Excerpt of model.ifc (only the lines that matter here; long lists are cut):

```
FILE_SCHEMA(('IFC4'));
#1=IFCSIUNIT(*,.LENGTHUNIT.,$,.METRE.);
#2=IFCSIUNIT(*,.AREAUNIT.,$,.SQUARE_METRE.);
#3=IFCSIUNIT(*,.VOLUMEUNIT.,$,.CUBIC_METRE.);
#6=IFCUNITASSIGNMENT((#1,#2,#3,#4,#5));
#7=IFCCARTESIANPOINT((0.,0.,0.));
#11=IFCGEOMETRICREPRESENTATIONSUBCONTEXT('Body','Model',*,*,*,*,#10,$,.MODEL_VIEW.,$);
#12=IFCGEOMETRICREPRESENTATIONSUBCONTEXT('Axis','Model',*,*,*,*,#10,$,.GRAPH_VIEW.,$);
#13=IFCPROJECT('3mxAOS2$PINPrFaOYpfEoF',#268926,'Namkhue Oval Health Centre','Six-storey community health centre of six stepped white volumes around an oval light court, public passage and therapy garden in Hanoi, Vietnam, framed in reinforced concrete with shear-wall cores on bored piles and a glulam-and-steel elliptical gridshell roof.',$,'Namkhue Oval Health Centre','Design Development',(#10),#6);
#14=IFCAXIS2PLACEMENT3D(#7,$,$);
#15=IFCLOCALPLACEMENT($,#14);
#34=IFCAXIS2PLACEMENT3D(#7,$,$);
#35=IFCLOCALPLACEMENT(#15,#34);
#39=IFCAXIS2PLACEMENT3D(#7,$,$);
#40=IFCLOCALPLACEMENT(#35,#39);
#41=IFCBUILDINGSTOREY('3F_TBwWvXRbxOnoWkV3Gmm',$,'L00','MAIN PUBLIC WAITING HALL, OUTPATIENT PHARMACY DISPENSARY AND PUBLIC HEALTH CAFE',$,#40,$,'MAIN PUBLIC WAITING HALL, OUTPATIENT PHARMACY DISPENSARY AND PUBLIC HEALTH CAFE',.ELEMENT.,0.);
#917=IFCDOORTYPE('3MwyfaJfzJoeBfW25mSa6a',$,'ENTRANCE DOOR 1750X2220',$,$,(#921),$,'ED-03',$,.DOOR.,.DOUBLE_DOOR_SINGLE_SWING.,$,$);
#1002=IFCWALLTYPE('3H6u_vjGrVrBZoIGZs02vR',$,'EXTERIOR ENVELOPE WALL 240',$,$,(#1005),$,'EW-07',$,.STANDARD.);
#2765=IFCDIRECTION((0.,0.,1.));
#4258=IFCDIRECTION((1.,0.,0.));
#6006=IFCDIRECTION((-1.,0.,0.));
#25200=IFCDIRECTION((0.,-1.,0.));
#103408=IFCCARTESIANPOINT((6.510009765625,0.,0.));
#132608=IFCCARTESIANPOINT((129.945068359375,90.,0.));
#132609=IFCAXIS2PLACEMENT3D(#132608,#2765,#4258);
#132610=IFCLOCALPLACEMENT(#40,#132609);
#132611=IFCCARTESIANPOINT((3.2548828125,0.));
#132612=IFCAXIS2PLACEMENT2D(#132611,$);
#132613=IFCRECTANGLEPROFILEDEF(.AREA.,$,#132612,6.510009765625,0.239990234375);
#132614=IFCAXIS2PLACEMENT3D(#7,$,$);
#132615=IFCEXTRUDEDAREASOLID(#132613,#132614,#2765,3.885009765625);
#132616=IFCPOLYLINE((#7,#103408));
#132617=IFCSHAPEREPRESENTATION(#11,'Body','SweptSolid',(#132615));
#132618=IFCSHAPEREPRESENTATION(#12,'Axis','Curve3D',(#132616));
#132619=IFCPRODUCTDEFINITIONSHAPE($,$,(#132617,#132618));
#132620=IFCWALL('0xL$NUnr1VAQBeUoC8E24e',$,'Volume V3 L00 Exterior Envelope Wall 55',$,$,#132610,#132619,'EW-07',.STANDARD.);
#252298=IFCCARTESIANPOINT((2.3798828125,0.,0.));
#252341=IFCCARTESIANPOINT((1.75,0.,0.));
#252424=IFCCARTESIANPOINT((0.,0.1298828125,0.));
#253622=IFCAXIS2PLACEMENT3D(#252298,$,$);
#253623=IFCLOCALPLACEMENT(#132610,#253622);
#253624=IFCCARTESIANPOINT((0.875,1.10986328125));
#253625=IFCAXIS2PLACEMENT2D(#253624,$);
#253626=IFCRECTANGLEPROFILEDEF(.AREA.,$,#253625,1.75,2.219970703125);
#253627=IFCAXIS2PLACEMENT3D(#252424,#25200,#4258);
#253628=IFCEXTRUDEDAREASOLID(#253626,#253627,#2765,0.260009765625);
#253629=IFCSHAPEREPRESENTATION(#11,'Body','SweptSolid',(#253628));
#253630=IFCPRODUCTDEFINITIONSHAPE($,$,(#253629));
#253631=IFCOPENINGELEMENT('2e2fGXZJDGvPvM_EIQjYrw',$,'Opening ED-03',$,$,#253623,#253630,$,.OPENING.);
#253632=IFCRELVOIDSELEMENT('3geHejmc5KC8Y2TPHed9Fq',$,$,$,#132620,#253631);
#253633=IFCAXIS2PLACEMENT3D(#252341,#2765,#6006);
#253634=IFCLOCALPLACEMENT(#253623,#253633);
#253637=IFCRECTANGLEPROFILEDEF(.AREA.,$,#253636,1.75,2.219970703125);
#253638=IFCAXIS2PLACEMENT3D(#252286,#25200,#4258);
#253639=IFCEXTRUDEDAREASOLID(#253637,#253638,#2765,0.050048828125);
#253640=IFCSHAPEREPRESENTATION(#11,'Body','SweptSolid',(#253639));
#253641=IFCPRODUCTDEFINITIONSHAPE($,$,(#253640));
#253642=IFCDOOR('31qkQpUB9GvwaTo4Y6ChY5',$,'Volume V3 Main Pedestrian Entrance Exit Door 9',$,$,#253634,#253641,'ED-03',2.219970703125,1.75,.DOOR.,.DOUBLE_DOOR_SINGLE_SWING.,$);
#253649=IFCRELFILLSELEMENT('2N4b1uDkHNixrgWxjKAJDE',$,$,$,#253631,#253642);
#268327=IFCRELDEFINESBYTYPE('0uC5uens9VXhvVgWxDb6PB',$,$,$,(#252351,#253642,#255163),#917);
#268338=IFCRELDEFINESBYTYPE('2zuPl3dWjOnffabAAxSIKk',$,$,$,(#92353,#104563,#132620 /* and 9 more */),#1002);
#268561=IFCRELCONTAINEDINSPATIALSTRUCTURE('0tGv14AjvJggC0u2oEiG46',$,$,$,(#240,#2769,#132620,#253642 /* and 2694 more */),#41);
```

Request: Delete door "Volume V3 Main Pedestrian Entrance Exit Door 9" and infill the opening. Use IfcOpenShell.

```python
import ifcopenshell
import ifcopenshell.api.feature
import ifcopenshell.api.root
import ifcopenshell.geom
import ifcopenshell.util.shape

model = ifcopenshell.open("model.ifc")
settings = ifcopenshell.geom.settings()


def volume(element):
    """Net volume in cubic metres, openings subtracted."""
    shape = ifcopenshell.geom.create_shape(settings, element)
    return ifcopenshell.util.shape.get_volume(shape.geometry)


door = model.by_guid("31qkQpUB9GvwaTo4Y6ChY5")
opening = door.FillsVoids[0].RelatingOpeningElement
wall = opening.VoidsElements[0].RelatingBuildingElement
before = volume(wall)

ifcopenshell.api.root.remove_product(model, product=door)
ifcopenshell.api.feature.remove_feature(model, feature=opening)

after = volume(wall)

print(f"wall volume {before:.3f} -> {after:.3f} m3")

model.write("model_edited.ifc")
```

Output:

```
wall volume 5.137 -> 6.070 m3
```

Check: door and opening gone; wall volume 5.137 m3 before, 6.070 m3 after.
